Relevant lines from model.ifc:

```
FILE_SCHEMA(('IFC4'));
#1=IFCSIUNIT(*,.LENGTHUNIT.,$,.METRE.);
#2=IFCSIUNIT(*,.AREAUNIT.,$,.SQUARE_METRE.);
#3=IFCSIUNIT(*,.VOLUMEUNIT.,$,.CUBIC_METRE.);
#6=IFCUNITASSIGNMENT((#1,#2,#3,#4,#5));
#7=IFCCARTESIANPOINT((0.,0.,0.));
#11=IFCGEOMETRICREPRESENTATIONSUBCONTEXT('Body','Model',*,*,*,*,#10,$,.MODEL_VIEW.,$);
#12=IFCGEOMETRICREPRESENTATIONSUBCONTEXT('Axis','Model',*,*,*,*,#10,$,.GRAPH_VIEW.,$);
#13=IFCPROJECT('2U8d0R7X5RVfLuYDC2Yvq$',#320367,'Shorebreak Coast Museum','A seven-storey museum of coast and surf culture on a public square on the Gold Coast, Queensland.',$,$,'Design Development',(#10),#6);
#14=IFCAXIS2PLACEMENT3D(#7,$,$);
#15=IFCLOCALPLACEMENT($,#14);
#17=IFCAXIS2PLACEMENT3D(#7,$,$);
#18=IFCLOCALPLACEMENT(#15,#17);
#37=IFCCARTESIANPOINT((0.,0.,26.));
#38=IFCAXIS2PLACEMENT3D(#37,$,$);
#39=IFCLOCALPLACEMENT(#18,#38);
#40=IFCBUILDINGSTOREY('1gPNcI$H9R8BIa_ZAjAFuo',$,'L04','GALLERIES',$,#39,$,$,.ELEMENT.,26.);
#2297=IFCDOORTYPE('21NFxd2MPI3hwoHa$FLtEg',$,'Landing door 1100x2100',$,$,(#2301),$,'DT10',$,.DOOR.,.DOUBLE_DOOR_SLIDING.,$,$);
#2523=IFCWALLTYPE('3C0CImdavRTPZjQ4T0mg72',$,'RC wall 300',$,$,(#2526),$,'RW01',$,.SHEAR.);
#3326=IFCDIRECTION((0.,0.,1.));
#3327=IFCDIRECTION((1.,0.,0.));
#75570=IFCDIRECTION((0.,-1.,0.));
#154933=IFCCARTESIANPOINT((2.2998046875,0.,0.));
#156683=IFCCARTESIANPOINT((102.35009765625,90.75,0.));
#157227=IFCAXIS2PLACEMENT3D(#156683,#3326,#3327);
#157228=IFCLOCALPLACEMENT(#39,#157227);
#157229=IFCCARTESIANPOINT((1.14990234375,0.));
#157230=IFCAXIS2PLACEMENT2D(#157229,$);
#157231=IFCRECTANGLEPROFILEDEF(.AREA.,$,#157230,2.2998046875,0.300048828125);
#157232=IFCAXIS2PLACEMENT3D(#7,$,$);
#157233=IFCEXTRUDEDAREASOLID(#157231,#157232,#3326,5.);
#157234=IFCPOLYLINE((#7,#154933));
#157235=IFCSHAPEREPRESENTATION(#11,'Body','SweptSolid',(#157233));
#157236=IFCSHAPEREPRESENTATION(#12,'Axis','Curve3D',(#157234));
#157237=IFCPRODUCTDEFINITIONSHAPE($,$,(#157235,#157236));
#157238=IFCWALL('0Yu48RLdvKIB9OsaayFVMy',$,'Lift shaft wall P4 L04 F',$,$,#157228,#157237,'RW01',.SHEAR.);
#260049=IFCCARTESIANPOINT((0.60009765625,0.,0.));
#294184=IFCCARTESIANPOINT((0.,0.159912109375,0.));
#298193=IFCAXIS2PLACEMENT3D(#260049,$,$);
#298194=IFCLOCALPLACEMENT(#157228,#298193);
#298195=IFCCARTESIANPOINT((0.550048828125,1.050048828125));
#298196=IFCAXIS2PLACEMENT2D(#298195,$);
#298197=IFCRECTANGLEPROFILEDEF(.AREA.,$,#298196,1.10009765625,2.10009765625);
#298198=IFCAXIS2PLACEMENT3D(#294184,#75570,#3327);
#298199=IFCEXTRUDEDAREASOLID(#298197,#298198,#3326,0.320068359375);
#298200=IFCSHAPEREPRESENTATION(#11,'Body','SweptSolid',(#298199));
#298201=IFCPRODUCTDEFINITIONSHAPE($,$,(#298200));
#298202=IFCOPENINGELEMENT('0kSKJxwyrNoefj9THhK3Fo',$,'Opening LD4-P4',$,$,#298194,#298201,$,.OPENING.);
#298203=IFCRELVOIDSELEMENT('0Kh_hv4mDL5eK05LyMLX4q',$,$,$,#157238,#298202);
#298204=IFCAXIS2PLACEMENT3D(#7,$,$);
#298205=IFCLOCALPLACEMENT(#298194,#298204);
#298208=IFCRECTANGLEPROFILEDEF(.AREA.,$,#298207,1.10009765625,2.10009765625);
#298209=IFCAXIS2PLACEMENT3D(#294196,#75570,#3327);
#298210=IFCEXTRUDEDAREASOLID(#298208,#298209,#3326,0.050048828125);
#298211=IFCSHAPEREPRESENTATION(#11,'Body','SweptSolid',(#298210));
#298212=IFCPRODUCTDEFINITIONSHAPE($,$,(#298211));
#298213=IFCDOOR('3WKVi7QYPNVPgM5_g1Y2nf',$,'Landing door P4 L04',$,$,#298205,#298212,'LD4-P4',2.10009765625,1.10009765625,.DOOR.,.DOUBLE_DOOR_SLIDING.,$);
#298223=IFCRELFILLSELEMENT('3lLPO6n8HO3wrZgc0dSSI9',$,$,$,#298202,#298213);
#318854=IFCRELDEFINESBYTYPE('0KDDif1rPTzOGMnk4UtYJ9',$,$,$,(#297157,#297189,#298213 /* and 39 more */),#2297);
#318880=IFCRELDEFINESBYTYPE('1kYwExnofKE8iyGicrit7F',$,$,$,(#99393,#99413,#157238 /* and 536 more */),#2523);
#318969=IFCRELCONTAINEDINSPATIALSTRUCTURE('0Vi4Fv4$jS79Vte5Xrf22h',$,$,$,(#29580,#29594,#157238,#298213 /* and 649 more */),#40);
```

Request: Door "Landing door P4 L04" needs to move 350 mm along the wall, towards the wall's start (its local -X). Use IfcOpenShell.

```python
import ifcopenshell
import ifcopenshell.api.geometry
import ifcopenshell.util.placement
import ifcopenshell.util.unit

model = ifcopenshell.open("model.ifc")
unit_scale = ifcopenshell.util.unit.calculate_unit_scale(model)

door = model.by_id(298213)
opening = door.FillsVoids[0].RelatingOpeningElement
wall = opening.VoidsElements[0].RelatingBuildingElement

wall_matrix = ifcopenshell.util.placement.get_local_placement(wall.ObjectPlacement)
shift = wall_matrix[:3, 0] * -0.35 / unit_scale
before = ifcopenshell.util.placement.get_local_placement(door.ObjectPlacement)[:3, 3].copy()

# The door is placed relative to its opening, so it follows when the opening moves.
matrix = ifcopenshell.util.placement.get_local_placement(opening.ObjectPlacement)
matrix[:3, 3] += shift
ifcopenshell.api.geometry.edit_object_placement(
    model, product=opening, matrix=matrix, is_si=False, should_transform_children=True
)

after = ifcopenshell.util.placement.get_local_placement(door.ObjectPlacement)[:3, 3]
print("door moved by", (after - before).round(3) + 0.0)

model.write("model_v2.ifc")
```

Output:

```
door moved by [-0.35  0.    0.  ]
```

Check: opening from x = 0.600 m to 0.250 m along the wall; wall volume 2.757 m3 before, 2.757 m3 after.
